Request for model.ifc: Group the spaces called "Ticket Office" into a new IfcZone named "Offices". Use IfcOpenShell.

First a look at what the model holds.

```python
import ifcopenshell

model = ifcopenshell.open("model.ifc")
print(model.schema)
seen = {}
for space in model.by_type("IfcSpace"):
    seen[space.LongName] = seen.get(space.LongName, 0) + 1
for name, count in sorted(seen.items(), key=str):
    print(count, "x", name)
print("zones:", [z.Name for z in model.by_type("IfcZone")][:20])
```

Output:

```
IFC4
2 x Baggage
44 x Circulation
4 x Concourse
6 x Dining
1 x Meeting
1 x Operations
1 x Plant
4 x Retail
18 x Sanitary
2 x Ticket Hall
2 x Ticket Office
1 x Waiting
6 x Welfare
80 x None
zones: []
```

```python
import ifcopenshell
import ifcopenshell.api.group
import ifcopenshell.api.root

model = ifcopenshell.open("model.ifc")

names = {"Ticket Office"}
spaces = [s for s in model.by_type("IfcSpace") if s.LongName in names]

zone = ifcopenshell.api.root.create_entity(model, ifc_class="IfcZone", name="Offices")
ifcopenshell.api.group.assign_group(model, products=spaces, group=zone)
print(len(spaces), "spaces in", zone.Name)

model.write("model_v2.ifc")
```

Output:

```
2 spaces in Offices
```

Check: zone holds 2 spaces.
